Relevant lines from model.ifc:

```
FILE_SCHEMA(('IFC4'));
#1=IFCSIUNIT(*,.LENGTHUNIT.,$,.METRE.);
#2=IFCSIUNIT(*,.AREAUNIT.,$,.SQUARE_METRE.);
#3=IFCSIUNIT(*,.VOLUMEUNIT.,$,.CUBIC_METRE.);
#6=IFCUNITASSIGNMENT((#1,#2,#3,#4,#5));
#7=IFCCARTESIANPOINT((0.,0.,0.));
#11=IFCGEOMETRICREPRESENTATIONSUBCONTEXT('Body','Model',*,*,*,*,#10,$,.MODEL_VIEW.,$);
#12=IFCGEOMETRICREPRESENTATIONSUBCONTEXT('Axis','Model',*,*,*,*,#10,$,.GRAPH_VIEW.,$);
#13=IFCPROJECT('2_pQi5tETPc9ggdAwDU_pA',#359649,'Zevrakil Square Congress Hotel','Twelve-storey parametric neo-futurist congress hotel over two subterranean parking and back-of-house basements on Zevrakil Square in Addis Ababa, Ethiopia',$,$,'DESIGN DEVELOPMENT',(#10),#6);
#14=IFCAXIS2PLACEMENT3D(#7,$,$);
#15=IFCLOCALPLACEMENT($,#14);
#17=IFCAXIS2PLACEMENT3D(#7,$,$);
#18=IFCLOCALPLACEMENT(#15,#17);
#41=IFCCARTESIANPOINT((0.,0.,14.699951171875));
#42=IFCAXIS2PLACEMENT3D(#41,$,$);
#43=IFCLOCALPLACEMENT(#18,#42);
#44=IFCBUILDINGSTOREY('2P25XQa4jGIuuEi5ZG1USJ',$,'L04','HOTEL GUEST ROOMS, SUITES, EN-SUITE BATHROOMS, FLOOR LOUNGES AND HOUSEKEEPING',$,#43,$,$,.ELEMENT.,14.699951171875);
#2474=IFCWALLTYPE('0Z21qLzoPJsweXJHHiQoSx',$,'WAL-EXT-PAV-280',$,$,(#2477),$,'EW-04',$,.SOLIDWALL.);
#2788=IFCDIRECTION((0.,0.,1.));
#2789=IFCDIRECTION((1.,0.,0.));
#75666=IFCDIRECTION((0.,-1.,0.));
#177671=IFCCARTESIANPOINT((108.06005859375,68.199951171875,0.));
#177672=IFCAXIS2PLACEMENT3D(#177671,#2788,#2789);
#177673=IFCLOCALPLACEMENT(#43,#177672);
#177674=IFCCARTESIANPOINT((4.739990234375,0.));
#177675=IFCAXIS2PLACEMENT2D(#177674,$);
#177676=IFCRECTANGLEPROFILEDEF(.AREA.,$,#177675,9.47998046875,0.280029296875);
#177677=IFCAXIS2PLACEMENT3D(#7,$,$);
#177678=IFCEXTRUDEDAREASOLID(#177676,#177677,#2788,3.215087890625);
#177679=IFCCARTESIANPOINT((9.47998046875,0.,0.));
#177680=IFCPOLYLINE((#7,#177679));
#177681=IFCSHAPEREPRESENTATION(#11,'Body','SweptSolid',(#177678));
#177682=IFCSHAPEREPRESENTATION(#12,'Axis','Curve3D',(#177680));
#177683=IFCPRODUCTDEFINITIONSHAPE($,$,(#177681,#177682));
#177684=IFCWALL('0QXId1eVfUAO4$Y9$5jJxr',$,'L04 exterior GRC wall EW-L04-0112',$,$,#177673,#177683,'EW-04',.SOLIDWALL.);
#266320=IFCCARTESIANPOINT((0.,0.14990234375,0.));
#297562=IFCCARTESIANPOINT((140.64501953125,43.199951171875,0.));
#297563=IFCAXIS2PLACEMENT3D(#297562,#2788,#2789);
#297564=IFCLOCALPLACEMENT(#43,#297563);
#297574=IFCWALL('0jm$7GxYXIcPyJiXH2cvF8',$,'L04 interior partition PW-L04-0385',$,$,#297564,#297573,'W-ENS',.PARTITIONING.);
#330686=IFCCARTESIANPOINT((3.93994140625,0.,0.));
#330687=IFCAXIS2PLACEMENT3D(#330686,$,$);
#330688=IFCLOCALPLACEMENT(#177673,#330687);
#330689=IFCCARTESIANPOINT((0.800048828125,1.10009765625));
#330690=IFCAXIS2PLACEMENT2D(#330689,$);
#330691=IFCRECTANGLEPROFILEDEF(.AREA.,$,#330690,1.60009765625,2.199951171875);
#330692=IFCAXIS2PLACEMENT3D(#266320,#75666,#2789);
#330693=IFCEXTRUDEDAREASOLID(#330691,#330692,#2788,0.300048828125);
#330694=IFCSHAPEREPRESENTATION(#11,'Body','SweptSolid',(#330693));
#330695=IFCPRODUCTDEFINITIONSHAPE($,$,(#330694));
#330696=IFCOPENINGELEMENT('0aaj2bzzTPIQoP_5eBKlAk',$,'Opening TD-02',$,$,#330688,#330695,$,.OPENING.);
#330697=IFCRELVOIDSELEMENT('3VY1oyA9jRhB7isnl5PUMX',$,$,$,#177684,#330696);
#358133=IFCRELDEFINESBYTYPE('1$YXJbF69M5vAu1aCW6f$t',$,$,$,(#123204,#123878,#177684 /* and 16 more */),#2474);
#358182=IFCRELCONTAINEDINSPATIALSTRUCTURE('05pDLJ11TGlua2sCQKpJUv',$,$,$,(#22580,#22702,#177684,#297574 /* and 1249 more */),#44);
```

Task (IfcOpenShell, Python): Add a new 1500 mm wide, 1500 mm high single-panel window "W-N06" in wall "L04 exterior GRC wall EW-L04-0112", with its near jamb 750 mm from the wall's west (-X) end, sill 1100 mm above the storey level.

```python
import numpy as np
import ifcopenshell
import ifcopenshell.api.feature
import ifcopenshell.api.geometry
import ifcopenshell.api.root
import ifcopenshell.api.spatial
import ifcopenshell.geom
import ifcopenshell.util.element
import ifcopenshell.util.placement
import ifcopenshell.util.representation
import ifcopenshell.util.shape
import ifcopenshell.util.unit

model = ifcopenshell.open("model.ifc")
unit_scale = ifcopenshell.util.unit.calculate_unit_scale(model)
settings = ifcopenshell.geom.settings()


def volume(element):
    """Net volume in cubic metres, openings subtracted."""
    shape = ifcopenshell.geom.create_shape(settings, element)
    return ifcopenshell.util.shape.get_volume(shape.geometry)


wall = model.by_guid("0QXId1eVfUAO4$Y9$5jJxr")
storey = ifcopenshell.util.element.get_container(wall, ifc_class="IfcBuildingStorey")
context = ifcopenshell.util.representation.get_context(model, "Model", "Body", "MODEL_VIEW")
before = volume(wall)

width, height, from_end, sill = 1.5, 1.5, 0.75, 1.1  # metres

# The wall runs along its own X axis, and the end named is its -X end.
wall_shape = ifcopenshell.geom.create_shape(settings, wall)
x, y, z = ifcopenshell.util.shape.get_vertices(wall_shape.geometry).T
start = x.min() + from_end
face, thickness = float(y.min()), float(y.max() - y.min())
wall_matrix = ifcopenshell.util.placement.get_local_placement(wall.ObjectPlacement)
level = ifcopenshell.util.placement.get_local_placement(storey.ObjectPlacement)[2, 3]


def in_wall(x, y):
    """Placement at x, y metres in the wall's axes, at sill height."""
    matrix = wall_matrix.copy()
    matrix[:, 3] = wall_matrix @ np.array([x / unit_scale, y / unit_scale, 0.0, 1.0])
    matrix[2, 3] = level + sill / unit_scale
    return matrix


# Opening: a box that overshoots both wall faces by 50 mm.
opening = ifcopenshell.api.root.create_entity(model, ifc_class="IfcOpeningElement", predefined_type="OPENING")
box = ifcopenshell.api.geometry.add_wall_representation(
    model, context=context, length=width, height=height, thickness=thickness + 0.1
)
ifcopenshell.api.geometry.assign_representation(model, product=opening, representation=box)
ifcopenshell.api.geometry.edit_object_placement(model, product=opening, matrix=in_wall(start, face - 0.05), is_si=False)
ifcopenshell.api.feature.add_feature(model, feature=opening, element=wall)

window = ifcopenshell.api.root.create_entity(model, ifc_class="IfcWindow", name="W-N06", predefined_type="WINDOW")
window.OverallWidth, window.OverallHeight = width / unit_scale, height / unit_scale
window.PartitioningType = "SINGLE_PANEL"
body = ifcopenshell.api.geometry.add_window_representation(
    model,
    context=context,
    overall_width=window.OverallWidth,
    overall_height=window.OverallHeight,
    partition_type="SINGLE_PANEL",
)
ifcopenshell.api.geometry.assign_representation(model, product=window, representation=body)
ifcopenshell.api.spatial.assign_container(model, products=[window], relating_structure=storey)
ifcopenshell.api.feature.add_filling(model, opening=opening, element=window)

# Centre the window in the wall's thickness.
ifcopenshell.api.geometry.edit_object_placement(model, product=window, matrix=in_wall(start, face), is_si=False)
window_shape = ifcopenshell.geom.create_shape(settings, window)
depth = ifcopenshell.util.shape.get_vertices(window_shape.geometry)[:, 1]
offset = face + thickness / 2 - (depth.min() + depth.max()) / 2
ifcopenshell.api.geometry.edit_object_placement(model, product=window, matrix=in_wall(start, offset), is_si=False)

after = volume(wall)

print(f"wall volume {before:.3f} -> {after:.3f} m3")

model.write("model_edited.ifc")
```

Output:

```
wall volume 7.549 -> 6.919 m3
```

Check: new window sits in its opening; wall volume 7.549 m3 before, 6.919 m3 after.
